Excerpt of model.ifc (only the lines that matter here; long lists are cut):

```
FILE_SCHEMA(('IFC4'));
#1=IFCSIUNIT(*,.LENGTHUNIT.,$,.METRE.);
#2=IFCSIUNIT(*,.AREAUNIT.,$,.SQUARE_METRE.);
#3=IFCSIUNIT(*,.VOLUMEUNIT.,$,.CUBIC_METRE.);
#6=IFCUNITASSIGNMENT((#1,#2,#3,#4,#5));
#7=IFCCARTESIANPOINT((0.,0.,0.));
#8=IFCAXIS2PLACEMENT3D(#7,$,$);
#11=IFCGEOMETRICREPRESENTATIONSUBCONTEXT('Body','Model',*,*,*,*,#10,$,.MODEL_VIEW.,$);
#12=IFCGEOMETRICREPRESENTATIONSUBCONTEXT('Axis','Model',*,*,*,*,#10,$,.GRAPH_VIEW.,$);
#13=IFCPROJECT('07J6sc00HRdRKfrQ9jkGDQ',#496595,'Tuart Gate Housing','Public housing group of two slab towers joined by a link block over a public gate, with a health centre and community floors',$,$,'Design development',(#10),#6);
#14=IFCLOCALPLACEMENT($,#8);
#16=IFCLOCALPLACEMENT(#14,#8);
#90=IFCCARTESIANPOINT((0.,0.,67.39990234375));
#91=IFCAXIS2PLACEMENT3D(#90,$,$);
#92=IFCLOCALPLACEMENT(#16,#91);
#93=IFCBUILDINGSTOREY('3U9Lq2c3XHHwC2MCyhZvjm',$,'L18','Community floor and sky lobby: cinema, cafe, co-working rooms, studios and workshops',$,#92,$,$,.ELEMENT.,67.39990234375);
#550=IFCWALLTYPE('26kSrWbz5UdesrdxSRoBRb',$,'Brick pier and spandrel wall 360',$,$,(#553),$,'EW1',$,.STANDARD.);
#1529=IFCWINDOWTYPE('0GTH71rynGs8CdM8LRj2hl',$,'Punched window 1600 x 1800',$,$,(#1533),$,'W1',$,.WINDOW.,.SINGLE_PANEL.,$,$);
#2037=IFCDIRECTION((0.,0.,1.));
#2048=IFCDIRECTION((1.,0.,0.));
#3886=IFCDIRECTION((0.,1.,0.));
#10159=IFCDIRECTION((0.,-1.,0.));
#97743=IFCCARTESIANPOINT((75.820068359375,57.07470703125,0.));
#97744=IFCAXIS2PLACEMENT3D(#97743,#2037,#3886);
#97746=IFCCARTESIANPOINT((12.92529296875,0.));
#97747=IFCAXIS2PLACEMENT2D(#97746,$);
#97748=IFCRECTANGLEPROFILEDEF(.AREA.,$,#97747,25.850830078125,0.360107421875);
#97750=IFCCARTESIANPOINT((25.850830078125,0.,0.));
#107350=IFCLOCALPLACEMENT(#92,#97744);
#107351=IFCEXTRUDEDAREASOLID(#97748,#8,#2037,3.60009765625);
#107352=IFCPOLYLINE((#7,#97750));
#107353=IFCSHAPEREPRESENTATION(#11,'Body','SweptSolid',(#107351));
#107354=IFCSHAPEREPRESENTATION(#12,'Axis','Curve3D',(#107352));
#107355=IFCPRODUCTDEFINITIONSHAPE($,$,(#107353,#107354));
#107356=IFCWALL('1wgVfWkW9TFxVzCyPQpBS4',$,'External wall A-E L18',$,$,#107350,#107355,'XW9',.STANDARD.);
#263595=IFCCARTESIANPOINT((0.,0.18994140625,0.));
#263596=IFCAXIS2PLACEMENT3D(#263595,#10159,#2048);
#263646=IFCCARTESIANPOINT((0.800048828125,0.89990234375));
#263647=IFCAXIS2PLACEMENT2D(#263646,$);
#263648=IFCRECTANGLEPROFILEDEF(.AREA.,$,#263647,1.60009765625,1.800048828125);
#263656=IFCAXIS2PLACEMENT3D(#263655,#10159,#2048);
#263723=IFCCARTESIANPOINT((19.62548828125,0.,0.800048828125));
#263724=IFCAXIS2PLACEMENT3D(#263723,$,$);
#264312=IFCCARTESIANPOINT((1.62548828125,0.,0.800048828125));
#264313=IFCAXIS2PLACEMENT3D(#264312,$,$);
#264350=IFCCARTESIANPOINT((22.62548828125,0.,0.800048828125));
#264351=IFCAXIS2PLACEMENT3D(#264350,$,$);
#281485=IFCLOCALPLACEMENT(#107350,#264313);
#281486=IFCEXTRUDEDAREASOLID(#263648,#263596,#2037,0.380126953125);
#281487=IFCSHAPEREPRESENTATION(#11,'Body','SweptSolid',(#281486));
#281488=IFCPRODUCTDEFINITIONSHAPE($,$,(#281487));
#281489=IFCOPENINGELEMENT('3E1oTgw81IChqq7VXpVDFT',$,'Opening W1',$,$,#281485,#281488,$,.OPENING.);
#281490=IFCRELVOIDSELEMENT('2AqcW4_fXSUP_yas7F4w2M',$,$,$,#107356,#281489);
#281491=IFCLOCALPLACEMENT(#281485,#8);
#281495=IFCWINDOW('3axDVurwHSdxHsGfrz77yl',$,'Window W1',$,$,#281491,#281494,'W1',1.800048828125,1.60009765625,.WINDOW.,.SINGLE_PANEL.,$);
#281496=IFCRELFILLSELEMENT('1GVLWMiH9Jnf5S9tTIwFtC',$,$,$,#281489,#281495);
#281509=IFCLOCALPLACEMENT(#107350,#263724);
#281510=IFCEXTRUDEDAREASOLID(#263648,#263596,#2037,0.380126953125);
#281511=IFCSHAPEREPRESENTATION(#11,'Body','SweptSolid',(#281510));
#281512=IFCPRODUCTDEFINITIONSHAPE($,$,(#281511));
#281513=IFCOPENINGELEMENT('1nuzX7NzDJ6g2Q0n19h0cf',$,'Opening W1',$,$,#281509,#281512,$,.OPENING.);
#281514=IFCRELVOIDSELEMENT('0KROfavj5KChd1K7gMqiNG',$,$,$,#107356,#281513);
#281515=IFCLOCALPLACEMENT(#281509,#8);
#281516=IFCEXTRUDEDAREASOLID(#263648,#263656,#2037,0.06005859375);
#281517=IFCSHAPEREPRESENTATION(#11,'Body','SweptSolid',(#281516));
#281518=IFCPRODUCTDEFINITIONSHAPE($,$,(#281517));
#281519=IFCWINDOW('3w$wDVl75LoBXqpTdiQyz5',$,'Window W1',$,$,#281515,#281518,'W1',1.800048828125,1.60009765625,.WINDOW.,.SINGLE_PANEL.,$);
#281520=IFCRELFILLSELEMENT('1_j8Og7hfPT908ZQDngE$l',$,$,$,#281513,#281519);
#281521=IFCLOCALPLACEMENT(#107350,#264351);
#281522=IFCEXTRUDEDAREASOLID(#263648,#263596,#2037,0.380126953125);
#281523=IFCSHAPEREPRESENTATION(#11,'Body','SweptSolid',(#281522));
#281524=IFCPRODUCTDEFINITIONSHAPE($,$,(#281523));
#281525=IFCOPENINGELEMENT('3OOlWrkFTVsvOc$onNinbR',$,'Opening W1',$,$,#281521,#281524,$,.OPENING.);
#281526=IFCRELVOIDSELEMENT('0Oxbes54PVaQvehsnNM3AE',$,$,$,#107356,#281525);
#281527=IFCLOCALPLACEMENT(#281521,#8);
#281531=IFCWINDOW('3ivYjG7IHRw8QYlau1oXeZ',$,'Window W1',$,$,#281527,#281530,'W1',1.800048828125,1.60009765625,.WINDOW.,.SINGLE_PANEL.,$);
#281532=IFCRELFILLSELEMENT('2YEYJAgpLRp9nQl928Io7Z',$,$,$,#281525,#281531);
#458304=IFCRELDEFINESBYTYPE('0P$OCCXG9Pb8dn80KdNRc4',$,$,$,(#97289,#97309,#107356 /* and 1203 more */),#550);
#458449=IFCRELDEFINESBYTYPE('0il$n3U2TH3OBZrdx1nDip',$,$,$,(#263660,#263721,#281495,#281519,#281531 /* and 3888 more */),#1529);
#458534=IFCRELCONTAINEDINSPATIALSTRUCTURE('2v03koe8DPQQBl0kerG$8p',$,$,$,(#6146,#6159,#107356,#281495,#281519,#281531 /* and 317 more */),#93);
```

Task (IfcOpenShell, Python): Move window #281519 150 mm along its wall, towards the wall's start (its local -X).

```python
import ifcopenshell
import ifcopenshell.api.geometry
import ifcopenshell.util.placement
import ifcopenshell.util.unit

model = ifcopenshell.open("model.ifc")
unit_scale = ifcopenshell.util.unit.calculate_unit_scale(model)

window = model.by_guid("3w$wDVl75LoBXqpTdiQyz5")
opening = window.FillsVoids[0].RelatingOpeningElement
wall = opening.VoidsElements[0].RelatingBuildingElement

wall_matrix = ifcopenshell.util.placement.get_local_placement(wall.ObjectPlacement)
shift = wall_matrix[:3, 0] * -0.15 / unit_scale
before = ifcopenshell.util.placement.get_local_placement(window.ObjectPlacement)[:3, 3].copy()

# The window is placed relative to its opening, so it follows when the opening moves.
matrix = ifcopenshell.util.placement.get_local_placement(opening.ObjectPlacement)
matrix[:3, 3] += shift
ifcopenshell.api.geometry.edit_object_placement(
    model, product=opening, matrix=matrix, is_si=False, should_transform_children=True
)

after = ifcopenshell.util.placement.get_local_placement(window.ObjectPlacement)[:3, 3]
print("window moved by", (after - before).round(3) + 0.0)

model.write("model_v2.ifc")
```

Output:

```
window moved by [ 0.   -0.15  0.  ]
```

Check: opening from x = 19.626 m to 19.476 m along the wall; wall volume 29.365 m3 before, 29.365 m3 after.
